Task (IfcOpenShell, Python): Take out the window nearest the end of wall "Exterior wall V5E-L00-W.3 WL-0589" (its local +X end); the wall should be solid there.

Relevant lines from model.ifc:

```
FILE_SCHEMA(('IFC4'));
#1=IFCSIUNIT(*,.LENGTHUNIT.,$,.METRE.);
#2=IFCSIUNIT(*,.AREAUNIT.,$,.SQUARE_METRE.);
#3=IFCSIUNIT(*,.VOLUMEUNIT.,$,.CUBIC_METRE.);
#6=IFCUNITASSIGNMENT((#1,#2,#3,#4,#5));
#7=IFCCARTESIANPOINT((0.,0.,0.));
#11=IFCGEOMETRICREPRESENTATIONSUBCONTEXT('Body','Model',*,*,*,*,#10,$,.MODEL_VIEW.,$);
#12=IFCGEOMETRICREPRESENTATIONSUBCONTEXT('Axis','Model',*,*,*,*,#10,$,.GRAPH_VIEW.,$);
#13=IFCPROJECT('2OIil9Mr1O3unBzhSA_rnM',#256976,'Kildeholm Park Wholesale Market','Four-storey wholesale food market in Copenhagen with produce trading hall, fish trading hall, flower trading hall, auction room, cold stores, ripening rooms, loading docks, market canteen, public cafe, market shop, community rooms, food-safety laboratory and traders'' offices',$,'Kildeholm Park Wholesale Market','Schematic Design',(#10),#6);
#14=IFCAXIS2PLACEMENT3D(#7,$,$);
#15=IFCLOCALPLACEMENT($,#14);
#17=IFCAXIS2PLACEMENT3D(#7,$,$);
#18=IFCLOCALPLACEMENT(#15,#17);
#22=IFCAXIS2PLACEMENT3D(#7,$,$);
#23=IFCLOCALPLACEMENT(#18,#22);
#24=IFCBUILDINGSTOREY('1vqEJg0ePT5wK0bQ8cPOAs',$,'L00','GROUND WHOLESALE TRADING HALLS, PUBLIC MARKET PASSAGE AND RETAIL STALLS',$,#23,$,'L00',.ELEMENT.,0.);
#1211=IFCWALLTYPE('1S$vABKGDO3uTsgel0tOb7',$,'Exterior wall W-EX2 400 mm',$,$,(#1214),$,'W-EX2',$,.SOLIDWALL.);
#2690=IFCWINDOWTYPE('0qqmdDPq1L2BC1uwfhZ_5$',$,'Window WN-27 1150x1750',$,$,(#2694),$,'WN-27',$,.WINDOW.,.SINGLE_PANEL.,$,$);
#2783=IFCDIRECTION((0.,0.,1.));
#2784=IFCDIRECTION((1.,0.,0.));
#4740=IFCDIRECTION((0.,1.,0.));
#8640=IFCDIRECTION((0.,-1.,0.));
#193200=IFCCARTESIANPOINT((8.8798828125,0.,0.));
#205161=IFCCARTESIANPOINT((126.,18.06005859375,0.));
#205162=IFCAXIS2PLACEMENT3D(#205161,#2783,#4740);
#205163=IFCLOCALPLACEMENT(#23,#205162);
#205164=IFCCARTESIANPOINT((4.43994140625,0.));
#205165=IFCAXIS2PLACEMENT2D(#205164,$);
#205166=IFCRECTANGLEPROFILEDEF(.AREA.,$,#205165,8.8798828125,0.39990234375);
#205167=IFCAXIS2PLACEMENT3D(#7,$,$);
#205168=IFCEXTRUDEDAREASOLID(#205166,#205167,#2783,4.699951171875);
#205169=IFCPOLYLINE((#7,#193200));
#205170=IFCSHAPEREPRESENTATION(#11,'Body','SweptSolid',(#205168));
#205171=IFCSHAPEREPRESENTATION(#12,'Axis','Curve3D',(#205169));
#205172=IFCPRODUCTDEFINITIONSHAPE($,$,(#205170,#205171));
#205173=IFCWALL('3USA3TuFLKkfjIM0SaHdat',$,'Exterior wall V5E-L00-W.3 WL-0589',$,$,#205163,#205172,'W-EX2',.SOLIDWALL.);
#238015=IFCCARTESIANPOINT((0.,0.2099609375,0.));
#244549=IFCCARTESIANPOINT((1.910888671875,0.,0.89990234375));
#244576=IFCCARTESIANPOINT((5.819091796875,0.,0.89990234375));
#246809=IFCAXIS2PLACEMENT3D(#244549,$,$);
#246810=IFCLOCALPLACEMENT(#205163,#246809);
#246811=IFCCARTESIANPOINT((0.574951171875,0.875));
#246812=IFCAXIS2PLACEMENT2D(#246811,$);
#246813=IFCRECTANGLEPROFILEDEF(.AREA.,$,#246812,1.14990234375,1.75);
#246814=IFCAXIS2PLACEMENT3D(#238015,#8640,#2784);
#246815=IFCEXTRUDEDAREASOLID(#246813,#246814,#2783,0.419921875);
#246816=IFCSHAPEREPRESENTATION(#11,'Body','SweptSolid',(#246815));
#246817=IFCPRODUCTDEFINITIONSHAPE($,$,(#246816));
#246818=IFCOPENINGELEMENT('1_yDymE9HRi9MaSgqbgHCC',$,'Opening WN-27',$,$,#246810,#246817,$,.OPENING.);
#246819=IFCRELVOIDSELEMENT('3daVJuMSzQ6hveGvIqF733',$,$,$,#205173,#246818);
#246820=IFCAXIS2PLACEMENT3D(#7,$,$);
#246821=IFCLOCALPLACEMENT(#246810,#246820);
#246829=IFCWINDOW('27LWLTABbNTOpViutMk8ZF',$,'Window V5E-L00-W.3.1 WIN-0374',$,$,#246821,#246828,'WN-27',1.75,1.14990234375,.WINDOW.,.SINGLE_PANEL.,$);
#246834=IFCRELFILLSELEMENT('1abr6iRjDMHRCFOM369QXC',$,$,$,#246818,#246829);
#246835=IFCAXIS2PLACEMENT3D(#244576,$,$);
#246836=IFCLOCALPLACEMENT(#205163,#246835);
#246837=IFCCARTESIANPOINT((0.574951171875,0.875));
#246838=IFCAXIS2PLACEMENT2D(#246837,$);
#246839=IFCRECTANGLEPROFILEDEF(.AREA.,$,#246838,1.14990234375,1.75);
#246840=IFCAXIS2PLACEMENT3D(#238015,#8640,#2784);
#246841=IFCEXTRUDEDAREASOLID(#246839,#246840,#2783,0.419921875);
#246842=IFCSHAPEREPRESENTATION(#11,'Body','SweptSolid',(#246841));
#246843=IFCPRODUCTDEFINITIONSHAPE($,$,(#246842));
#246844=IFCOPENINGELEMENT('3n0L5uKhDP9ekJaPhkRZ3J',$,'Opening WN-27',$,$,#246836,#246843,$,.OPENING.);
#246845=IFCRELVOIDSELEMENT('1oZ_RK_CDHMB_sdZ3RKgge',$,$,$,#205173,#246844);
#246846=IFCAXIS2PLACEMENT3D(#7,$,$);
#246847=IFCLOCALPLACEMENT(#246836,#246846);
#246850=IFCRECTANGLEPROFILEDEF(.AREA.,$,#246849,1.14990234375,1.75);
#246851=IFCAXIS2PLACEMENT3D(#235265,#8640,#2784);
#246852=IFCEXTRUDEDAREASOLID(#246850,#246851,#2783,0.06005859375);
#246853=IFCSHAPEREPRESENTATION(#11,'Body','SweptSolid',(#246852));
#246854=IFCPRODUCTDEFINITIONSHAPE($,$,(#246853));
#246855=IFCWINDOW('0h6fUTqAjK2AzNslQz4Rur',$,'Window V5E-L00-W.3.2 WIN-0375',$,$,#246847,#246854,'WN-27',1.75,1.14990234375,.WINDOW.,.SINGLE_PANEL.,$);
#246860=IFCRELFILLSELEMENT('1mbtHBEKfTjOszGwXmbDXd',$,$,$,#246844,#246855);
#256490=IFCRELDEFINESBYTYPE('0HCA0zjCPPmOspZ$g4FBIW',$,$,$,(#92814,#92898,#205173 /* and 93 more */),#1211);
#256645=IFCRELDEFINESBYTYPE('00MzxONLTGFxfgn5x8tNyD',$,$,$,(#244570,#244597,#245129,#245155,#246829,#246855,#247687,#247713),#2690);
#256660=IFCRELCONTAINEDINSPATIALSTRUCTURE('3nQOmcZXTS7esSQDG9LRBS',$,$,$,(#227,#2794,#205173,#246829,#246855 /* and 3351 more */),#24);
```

```python
import ifcopenshell
import ifcopenshell.api.feature
import ifcopenshell.api.root
import ifcopenshell.geom
import ifcopenshell.util.shape

model = ifcopenshell.open("model.ifc")
settings = ifcopenshell.geom.settings()


def volume(element):
    """Net volume in cubic metres, openings subtracted."""
    shape = ifcopenshell.geom.create_shape(settings, element)
    return ifcopenshell.util.shape.get_volume(shape.geometry)


window = model.by_id(246855)
opening = window.FillsVoids[0].RelatingOpeningElement
wall = opening.VoidsElements[0].RelatingBuildingElement
before = volume(wall)

ifcopenshell.api.root.remove_product(model, product=window)
ifcopenshell.api.feature.remove_feature(model, feature=opening)

after = volume(wall)

print(f"wall volume {before:.3f} -> {after:.3f} m3")

model.write("model-out.ifc")
```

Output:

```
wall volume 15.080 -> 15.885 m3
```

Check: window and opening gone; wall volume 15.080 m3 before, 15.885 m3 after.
